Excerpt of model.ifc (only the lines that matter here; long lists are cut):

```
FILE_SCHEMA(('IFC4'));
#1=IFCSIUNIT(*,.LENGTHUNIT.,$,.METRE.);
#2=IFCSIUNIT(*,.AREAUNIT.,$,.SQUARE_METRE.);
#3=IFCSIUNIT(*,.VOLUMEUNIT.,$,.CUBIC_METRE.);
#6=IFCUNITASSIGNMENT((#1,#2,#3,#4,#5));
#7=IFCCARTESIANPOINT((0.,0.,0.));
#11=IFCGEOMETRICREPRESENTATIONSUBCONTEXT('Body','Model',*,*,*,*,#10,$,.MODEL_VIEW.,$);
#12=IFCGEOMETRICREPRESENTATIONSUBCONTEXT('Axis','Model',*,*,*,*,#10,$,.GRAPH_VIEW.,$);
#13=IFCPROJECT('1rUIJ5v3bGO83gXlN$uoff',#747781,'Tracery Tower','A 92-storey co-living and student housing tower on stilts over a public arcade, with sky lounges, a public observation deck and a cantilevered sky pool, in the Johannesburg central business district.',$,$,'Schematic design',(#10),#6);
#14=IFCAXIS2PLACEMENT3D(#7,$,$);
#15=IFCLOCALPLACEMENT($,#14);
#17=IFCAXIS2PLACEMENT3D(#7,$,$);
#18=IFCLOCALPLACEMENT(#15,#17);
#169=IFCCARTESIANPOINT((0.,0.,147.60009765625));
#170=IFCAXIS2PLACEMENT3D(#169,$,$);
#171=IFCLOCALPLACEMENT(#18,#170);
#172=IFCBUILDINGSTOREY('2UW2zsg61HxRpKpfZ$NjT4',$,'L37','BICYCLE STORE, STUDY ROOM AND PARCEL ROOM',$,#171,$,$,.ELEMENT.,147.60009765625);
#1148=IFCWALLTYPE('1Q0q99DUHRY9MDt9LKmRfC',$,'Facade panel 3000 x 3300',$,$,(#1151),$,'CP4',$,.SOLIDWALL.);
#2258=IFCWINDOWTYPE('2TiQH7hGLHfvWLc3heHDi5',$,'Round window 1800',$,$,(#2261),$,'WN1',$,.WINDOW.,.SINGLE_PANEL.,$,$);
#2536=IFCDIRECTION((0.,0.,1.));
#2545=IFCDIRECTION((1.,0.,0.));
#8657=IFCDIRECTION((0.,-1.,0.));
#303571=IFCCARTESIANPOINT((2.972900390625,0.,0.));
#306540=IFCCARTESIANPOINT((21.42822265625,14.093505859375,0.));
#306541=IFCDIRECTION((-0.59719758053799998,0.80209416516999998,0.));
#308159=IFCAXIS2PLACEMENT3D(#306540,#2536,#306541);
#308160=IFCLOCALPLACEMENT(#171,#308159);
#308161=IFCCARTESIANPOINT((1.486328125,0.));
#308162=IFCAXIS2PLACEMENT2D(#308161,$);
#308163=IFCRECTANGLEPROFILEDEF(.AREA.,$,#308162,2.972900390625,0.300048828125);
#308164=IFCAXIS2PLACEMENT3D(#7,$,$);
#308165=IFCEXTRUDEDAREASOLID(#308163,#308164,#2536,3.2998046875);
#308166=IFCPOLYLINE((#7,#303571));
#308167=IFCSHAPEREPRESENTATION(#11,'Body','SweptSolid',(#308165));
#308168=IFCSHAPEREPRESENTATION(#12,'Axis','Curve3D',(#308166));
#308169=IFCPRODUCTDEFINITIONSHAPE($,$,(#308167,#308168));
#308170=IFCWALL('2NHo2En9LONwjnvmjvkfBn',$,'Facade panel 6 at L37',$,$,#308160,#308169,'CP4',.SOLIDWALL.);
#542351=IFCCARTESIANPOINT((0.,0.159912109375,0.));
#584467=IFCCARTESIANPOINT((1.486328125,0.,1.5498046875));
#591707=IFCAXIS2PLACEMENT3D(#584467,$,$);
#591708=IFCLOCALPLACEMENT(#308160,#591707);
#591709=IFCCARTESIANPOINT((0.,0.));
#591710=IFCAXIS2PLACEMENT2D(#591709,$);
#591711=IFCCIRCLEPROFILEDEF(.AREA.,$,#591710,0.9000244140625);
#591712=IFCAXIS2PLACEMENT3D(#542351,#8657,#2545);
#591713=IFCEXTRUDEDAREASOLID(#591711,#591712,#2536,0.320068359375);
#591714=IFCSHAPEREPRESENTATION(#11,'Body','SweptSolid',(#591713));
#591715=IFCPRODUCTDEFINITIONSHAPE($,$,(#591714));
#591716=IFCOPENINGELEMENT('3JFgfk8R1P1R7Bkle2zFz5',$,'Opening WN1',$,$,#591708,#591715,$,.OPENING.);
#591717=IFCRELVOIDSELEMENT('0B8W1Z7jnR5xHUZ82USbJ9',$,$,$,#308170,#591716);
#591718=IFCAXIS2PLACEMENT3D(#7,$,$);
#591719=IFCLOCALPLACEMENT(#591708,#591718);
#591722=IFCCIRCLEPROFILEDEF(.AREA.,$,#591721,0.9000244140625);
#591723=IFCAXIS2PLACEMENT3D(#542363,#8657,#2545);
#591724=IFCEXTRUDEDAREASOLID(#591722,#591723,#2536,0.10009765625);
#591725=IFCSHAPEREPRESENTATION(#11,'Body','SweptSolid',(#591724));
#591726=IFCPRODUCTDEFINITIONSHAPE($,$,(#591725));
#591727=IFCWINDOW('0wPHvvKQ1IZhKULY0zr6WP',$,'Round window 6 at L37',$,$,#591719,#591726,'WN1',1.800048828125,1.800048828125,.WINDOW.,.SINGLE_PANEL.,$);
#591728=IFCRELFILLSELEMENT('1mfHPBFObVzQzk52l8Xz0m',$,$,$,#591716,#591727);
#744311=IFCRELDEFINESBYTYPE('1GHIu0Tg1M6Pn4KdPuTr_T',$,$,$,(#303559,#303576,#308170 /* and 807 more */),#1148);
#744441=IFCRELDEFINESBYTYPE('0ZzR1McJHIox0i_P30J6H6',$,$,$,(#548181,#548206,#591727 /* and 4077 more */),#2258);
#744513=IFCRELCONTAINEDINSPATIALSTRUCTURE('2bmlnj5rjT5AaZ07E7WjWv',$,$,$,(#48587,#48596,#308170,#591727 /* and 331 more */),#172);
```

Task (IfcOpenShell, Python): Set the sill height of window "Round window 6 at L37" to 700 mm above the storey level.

```python
import numpy as np
import ifcopenshell
import ifcopenshell.api.geometry
import ifcopenshell.geom
import ifcopenshell.util.element
import ifcopenshell.util.placement
import ifcopenshell.util.shape
import ifcopenshell.util.unit

model = ifcopenshell.open("model.ifc")
unit_scale = ifcopenshell.util.unit.calculate_unit_scale(model)

window = model.by_id(591727)
opening = window.FillsVoids[0].RelatingOpeningElement
storey = ifcopenshell.util.element.get_container(window, ifc_class="IfcBuildingStorey")
level = ifcopenshell.util.placement.get_local_placement(storey.ObjectPlacement)[2, 3]

# The opening's origin need not be at the sill, so measure its lowest point.
shape = ifcopenshell.geom.create_shape(ifcopenshell.geom.settings(), opening)
bottom = ifcopenshell.util.shape.get_shape_bottom_elevation(shape, shape.geometry) / unit_scale
dz = level + 0.7 - bottom

shift = np.array([0.0, 0.0, dz])
# The window is placed relative to its opening, so it follows when the opening moves.
matrix = ifcopenshell.util.placement.get_local_placement(opening.ObjectPlacement)
matrix[:3, 3] += shift
ifcopenshell.api.geometry.edit_object_placement(
    model, product=opening, matrix=matrix, is_si=False, should_transform_children=True
)

print(f"moved by {dz * unit_scale:+.3f} m")

model.write("model_updated.ifc")
```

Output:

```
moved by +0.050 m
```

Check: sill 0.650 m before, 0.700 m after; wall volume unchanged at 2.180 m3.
